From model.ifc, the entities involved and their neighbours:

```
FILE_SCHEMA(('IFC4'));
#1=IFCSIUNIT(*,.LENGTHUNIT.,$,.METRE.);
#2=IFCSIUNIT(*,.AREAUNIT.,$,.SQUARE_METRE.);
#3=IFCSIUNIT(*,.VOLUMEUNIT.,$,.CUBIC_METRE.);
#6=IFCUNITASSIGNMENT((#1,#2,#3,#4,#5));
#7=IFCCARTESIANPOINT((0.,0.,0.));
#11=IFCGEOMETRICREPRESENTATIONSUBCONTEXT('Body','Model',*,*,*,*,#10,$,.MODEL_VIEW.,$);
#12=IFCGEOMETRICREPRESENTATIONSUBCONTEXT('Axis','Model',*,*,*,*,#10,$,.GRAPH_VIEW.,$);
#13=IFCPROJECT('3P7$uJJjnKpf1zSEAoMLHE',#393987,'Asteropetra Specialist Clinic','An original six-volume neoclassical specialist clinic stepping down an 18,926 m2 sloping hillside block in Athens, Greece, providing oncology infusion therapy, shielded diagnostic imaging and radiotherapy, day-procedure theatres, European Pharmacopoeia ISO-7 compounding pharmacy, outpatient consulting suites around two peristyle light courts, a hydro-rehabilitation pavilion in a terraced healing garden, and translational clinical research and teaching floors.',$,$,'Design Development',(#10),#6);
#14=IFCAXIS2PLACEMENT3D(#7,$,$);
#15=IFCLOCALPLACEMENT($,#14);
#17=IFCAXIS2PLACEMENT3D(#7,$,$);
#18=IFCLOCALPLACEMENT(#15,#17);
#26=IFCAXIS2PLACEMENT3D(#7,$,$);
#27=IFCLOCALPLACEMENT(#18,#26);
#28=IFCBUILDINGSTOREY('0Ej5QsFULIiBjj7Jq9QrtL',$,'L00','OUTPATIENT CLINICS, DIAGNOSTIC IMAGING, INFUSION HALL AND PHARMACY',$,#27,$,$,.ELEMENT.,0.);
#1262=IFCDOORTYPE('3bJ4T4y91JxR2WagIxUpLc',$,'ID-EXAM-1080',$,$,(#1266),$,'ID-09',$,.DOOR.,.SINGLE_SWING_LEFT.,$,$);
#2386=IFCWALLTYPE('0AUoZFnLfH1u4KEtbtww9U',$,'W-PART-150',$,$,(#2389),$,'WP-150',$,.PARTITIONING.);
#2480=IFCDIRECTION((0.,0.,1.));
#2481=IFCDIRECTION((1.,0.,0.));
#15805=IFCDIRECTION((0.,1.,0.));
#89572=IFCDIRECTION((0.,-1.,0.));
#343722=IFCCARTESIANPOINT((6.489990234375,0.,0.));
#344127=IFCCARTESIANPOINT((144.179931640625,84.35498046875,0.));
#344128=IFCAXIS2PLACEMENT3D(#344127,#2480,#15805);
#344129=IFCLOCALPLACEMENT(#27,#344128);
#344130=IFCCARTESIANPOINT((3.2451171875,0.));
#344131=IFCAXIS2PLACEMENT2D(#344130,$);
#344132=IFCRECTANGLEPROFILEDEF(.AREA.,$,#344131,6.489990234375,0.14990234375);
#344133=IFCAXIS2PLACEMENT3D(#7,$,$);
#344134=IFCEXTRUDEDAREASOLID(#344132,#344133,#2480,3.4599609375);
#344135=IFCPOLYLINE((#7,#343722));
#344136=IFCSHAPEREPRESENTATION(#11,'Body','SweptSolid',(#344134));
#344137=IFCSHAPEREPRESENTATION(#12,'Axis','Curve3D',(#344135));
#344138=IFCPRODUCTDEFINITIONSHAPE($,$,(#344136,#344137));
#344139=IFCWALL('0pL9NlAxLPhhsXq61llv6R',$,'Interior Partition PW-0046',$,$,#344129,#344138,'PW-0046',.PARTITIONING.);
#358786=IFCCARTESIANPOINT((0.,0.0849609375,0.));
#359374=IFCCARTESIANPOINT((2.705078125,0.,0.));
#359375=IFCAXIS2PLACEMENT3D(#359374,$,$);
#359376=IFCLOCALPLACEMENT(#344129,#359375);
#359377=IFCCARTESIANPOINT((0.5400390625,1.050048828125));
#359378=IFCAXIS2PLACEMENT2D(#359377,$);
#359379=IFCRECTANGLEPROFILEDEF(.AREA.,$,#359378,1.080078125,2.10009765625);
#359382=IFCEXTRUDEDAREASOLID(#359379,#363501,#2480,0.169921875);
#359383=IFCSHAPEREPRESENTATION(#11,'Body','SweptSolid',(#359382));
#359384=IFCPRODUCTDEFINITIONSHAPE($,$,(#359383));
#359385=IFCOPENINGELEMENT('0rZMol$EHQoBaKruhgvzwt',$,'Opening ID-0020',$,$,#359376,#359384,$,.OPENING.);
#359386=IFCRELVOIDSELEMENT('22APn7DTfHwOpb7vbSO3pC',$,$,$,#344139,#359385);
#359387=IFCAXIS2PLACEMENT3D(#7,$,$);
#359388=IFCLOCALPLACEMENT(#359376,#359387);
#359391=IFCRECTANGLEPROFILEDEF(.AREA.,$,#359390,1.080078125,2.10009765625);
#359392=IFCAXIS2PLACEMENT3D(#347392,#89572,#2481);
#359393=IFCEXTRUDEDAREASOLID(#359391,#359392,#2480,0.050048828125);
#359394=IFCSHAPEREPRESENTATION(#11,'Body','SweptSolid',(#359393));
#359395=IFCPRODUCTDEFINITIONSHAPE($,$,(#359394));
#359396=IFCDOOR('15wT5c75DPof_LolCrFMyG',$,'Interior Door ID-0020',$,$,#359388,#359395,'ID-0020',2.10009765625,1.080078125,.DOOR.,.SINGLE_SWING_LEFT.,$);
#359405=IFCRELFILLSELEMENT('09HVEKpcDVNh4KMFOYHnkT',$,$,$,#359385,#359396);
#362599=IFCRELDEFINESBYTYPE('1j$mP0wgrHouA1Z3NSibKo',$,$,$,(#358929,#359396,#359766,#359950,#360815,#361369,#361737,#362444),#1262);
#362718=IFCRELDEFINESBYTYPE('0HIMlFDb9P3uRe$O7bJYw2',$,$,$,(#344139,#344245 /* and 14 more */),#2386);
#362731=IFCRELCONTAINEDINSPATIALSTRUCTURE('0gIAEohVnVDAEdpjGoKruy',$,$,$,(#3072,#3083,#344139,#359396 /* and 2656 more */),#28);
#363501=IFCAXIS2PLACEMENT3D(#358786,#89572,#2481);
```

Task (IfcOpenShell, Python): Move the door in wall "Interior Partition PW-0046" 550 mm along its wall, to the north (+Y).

```python
import ifcopenshell
import ifcopenshell.api.geometry
import ifcopenshell.util.placement

model = ifcopenshell.open("model.ifc")

door = model.by_id(359396)
opening = door.FillsVoids[0].RelatingOpeningElement
wall = opening.VoidsElements[0].RelatingBuildingElement

wall_matrix = ifcopenshell.util.placement.get_local_placement(wall.ObjectPlacement)
shift = wall_matrix[:3, 0] * 0.55
before = ifcopenshell.util.placement.get_local_placement(door.ObjectPlacement)[:3, 3].copy()

# The door is placed relative to its opening, so it follows when the opening moves.
matrix = ifcopenshell.util.placement.get_local_placement(opening.ObjectPlacement)
matrix[:3, 3] += shift
ifcopenshell.api.geometry.edit_object_placement(
    model, product=opening, matrix=matrix, is_si=False, should_transform_children=True
)

after = ifcopenshell.util.placement.get_local_placement(door.ObjectPlacement)[:3, 3]
print("door moved by", (after - before).round(3) + 0.0)

model.write("model-out.ifc")
```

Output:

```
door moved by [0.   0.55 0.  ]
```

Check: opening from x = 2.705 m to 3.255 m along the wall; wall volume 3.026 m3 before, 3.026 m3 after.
